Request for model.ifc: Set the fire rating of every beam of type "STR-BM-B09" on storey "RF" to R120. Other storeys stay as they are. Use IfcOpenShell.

First a look at what the model holds.

```python
import ifcopenshell
import ifcopenshell.util.element

model = ifcopenshell.open("model.ifc")
print(model.schema)
storey = next(s for s in model.by_type("IfcBuildingStorey") if s.Name == "RF")
beams = [e for e in ifcopenshell.util.element.get_decomposition(storey) if e.is_a("IfcBeam")]
seen = {}
for e in beams:
    element_type = ifcopenshell.util.element.get_type(e)
    key = (element_type.Name if element_type != e and element_type else None, ifcopenshell.util.element.get_pset(e, "Pset_BeamCommon", "FireRating"))
    seen[key] = seen.get(key, 0) + 1
for (name, value), count in sorted(seen.items(), key=str):
    print(count, "x", name, "|", value)
```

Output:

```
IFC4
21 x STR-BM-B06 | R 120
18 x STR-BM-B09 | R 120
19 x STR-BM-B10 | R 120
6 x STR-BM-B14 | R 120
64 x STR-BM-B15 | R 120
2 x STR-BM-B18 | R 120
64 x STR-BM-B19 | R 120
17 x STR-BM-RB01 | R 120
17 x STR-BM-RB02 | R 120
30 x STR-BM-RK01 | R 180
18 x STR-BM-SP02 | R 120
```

```python
import ifcopenshell
import ifcopenshell.api.pset
import ifcopenshell.util.element

model = ifcopenshell.open("model.ifc")

storey = next(s for s in model.by_type("IfcBuildingStorey") if s.Name == "RF")
beams = [e for e in ifcopenshell.util.element.get_decomposition(storey) if e.is_a("IfcBeam")]

count = 0
for e in beams:
    element_type = ifcopenshell.util.element.get_type(e)
    if element_type in (None, e) or element_type.Name != "STR-BM-B09":
        continue
    # add_pset returns the element's existing set when there is one.
    pset = ifcopenshell.api.pset.add_pset(model, product=e, name="Pset_BeamCommon")
    ifcopenshell.api.pset.edit_pset(model, pset=pset, properties={"FireRating": "R120"})
    count += 1

print(count, "beams updated")

model.write("model_v2.ifc")
```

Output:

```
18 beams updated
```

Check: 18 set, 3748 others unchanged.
